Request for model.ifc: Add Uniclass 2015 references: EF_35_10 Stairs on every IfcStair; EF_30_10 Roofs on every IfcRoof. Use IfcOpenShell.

First a look at what the model holds.

```python
import ifcopenshell

model = ifcopenshell.open("model.ifc")
print(model.schema)
print("classifications:", [c.Name for c in model.by_type("IfcClassification")])
for ifc_class in ("IfcDoor", "IfcRoof", "IfcStair", "IfcWall", "IfcWindow"):
    print(ifc_class, len(model.by_type(ifc_class)))
```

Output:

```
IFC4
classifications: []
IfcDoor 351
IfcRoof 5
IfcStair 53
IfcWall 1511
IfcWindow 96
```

```python
import ifcopenshell
import ifcopenshell.api.classification

model = ifcopenshell.open("model.ifc")

system = ifcopenshell.api.classification.add_classification(model, classification="Uniclass 2015")

codes = {
    "IfcStair": ("EF_35_10", "Stairs"),
    "IfcRoof": ("EF_30_10", "Roofs"),
}
for ifc_class, (code, name) in codes.items():
    products = model.by_type(ifc_class)
    ifcopenshell.api.classification.add_reference(
        model, products=products, classification=system, identification=code, name=name
    )
    print(code, len(products))

model.write("model_edited.ifc")
```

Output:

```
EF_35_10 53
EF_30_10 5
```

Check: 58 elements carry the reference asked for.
